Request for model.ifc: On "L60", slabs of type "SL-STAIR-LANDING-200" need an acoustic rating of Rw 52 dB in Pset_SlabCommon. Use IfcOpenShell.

First a look at what the model holds.

```python
import ifcopenshell
import ifcopenshell.util.element

model = ifcopenshell.open("model.ifc")
print(model.schema)
storey = next(s for s in model.by_type("IfcBuildingStorey") if s.Name == "L60")
slabs = [e for e in ifcopenshell.util.element.get_decomposition(storey) if e.is_a("IfcSlab")]
seen = {}
for e in slabs:
    element_type = ifcopenshell.util.element.get_type(e)
    key = (element_type.Name if element_type != e and element_type else None, ifcopenshell.util.element.get_pset(e, "Pset_SlabCommon", "AcousticRating"))
    seen[key] = seen.get(key, 0) + 1
for (name, value), count in sorted(seen.items(), key=str):
    print(count, "x", name, "|", value)
```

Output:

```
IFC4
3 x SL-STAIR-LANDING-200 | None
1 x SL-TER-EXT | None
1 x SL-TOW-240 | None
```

```python
import ifcopenshell
import ifcopenshell.api.pset
import ifcopenshell.util.element

model = ifcopenshell.open("model.ifc")

storey = next(s for s in model.by_type("IfcBuildingStorey") if s.Name == "L60")
slabs = [e for e in ifcopenshell.util.element.get_decomposition(storey) if e.is_a("IfcSlab")]

count = 0
for e in slabs:
    element_type = ifcopenshell.util.element.get_type(e)
    if element_type in (None, e) or element_type.Name != "SL-STAIR-LANDING-200":
        continue
    # add_pset returns the element's existing set when there is one.
    pset = ifcopenshell.api.pset.add_pset(model, product=e, name="Pset_SlabCommon")
    ifcopenshell.api.pset.edit_pset(model, pset=pset, properties={"AcousticRating": "Rw 52 dB"})
    count += 1

print(count, "slabs updated")

model.write("model-out.ifc")
```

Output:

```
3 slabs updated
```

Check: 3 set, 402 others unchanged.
